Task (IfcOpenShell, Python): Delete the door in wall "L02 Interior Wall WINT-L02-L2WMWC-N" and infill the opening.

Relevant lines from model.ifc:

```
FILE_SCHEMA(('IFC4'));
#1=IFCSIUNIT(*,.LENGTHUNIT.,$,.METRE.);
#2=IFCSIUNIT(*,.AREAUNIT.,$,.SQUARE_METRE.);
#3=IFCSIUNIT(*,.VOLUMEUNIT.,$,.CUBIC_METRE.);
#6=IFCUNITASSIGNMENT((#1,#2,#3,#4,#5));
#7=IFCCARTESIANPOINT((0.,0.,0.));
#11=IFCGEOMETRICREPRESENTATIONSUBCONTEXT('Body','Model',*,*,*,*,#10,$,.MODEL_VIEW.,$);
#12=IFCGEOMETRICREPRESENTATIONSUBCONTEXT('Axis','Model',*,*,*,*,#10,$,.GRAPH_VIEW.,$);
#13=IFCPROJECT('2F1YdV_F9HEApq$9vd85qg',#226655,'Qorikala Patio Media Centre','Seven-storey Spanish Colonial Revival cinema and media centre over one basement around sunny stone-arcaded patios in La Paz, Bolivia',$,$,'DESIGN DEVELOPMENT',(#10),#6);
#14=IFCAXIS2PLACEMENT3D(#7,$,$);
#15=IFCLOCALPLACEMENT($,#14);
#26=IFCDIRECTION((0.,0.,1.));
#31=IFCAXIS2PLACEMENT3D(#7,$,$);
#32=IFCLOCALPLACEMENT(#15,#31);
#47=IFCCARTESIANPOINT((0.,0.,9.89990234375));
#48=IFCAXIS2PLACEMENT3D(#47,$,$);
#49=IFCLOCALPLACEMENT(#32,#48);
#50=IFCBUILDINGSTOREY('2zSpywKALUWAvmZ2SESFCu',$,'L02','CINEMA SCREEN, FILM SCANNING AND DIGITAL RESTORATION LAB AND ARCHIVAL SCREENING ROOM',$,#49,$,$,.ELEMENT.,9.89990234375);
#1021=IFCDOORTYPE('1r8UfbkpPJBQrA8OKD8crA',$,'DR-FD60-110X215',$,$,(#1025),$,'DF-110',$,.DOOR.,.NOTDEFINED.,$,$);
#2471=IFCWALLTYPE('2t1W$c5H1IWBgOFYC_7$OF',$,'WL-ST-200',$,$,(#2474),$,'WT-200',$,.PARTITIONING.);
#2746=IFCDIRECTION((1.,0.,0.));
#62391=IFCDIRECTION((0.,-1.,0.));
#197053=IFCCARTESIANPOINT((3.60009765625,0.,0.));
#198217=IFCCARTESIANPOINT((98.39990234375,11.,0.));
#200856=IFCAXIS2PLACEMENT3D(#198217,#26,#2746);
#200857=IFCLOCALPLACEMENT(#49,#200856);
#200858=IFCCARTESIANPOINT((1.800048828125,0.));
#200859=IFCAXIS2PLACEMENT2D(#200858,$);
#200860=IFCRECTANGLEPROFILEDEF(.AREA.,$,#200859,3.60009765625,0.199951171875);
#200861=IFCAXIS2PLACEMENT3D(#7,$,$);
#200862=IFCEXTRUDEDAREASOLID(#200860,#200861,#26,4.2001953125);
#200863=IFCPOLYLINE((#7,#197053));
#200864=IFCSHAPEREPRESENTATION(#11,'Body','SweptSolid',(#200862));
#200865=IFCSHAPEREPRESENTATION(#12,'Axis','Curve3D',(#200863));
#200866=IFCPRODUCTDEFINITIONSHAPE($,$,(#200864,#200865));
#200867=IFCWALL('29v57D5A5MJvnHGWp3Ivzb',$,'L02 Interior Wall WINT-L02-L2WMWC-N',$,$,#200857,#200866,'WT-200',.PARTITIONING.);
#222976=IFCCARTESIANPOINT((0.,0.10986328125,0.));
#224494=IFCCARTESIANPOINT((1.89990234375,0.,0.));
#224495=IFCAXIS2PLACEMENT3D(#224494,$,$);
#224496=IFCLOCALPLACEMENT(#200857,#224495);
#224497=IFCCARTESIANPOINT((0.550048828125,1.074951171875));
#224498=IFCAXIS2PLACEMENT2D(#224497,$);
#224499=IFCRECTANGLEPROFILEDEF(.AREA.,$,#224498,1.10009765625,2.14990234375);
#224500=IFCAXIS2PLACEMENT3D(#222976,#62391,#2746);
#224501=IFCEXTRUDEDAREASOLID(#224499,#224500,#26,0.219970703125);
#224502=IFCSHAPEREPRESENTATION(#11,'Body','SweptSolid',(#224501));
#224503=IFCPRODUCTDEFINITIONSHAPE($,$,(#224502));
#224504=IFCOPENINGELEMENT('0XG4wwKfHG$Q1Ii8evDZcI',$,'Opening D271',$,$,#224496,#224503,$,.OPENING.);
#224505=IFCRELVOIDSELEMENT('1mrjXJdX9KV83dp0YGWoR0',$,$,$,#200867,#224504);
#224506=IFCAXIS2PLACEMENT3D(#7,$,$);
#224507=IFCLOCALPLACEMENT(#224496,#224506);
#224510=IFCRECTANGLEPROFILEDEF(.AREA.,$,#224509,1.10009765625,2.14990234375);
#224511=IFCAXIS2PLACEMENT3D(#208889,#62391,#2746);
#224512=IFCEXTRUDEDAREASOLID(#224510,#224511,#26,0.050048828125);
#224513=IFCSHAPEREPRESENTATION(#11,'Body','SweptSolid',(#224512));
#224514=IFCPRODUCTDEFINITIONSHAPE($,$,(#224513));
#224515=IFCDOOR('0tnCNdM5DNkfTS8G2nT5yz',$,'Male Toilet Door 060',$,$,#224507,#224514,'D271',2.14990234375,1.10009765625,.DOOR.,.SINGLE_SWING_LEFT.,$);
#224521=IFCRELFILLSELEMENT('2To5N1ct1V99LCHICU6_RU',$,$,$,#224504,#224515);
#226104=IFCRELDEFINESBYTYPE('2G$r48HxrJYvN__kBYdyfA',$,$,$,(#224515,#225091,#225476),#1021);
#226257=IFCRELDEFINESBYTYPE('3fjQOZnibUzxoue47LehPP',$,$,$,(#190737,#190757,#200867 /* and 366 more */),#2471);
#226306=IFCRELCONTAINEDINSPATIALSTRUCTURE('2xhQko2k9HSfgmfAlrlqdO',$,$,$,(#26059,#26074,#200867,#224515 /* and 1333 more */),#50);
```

```python
import ifcopenshell
import ifcopenshell.api.feature
import ifcopenshell.api.root
import ifcopenshell.geom
import ifcopenshell.util.shape

model = ifcopenshell.open("model.ifc")
settings = ifcopenshell.geom.settings()


def volume(element):
    """Net volume in cubic metres, openings subtracted."""
    shape = ifcopenshell.geom.create_shape(settings, element)
    return ifcopenshell.util.shape.get_volume(shape.geometry)


door = model.by_guid("0tnCNdM5DNkfTS8G2nT5yz")
opening = door.FillsVoids[0].RelatingOpeningElement
wall = opening.VoidsElements[0].RelatingBuildingElement
before = volume(wall)

ifcopenshell.api.root.remove_product(model, product=door)
ifcopenshell.api.feature.remove_feature(model, feature=opening)

after = volume(wall)

print(f"wall volume {before:.3f} -> {after:.3f} m3")

model.write("model_rev.ifc")
```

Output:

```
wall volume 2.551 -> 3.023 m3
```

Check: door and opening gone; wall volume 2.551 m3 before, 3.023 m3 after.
